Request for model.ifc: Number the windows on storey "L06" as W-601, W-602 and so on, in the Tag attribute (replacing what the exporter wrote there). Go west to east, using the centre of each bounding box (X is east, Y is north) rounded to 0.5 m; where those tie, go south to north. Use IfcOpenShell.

First a look at what the model holds.

```python
import ifcopenshell
import ifcopenshell.util.element
import ifcopenshell.util.placement

model = ifcopenshell.open("model.ifc")
print(model.schema)
storey = next(s for s in model.by_type("IfcBuildingStorey") if s.Name == "L06")
windows = [e for e in ifcopenshell.util.element.get_decomposition(storey) if e.is_a("IfcWindow")]
for e in sorted(windows, key=lambda e: e.id()):
    origin = ifcopenshell.util.placement.get_local_placement(e.ObjectPlacement)[:3, 3]
    print(e.id(), e.Tag, e.Name, origin.round(2) + 0.0, sep=" | ")
```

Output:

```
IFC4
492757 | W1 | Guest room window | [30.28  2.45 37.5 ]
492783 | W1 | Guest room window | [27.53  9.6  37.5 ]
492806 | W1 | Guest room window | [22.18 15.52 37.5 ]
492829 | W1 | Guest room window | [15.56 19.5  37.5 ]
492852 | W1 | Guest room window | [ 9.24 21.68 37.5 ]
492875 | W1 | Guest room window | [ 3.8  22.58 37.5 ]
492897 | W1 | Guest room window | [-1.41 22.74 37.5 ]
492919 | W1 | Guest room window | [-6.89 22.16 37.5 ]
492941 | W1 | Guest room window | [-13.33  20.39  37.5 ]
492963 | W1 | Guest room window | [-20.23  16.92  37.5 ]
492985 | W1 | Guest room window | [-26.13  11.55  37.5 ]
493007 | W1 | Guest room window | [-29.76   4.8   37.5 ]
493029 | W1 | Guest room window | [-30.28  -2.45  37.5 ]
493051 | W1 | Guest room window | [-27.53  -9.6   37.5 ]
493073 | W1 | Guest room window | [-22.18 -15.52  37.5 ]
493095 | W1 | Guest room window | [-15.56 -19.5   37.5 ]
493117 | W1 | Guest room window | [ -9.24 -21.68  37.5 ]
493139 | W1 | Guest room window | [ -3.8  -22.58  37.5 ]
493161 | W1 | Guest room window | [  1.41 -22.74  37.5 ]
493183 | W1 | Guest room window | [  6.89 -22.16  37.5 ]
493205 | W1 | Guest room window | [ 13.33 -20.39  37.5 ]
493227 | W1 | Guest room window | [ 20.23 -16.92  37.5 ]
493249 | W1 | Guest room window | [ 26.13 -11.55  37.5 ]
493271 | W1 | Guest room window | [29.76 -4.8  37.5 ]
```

```python
import ifcopenshell
import ifcopenshell.geom
import ifcopenshell.util.element
import ifcopenshell.util.shape

model = ifcopenshell.open("model.ifc")
settings = ifcopenshell.geom.settings()
settings.set("use-world-coords", True)


def centre(element):
    shape = ifcopenshell.geom.create_shape(settings, element)
    return ifcopenshell.util.shape.get_bbox_centroid(shape.geometry)


storey = next(s for s in model.by_type("IfcBuildingStorey") if s.Name == "L06")
windows = [e for e in ifcopenshell.util.element.get_decomposition(storey) if e.is_a("IfcWindow")]

# Insertion points can sit at a corner or the storey origin, so sort by the geometry (in metres).
centres = {e: centre(e) for e in windows}
windows.sort(key=lambda e: (round(centres[e][0] / 0.5), centres[e][1]))

for i, e in enumerate(windows, start=1):
    number = f"W-6{i:02d}"
    e.Tag = number
    print(e.id(), number)

model.write("model_rev.ifc")
```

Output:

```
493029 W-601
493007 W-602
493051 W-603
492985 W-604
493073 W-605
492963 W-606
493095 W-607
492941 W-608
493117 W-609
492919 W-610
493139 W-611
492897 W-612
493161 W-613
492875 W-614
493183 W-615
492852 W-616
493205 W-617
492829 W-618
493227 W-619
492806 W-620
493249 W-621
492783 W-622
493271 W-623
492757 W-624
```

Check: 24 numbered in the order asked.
